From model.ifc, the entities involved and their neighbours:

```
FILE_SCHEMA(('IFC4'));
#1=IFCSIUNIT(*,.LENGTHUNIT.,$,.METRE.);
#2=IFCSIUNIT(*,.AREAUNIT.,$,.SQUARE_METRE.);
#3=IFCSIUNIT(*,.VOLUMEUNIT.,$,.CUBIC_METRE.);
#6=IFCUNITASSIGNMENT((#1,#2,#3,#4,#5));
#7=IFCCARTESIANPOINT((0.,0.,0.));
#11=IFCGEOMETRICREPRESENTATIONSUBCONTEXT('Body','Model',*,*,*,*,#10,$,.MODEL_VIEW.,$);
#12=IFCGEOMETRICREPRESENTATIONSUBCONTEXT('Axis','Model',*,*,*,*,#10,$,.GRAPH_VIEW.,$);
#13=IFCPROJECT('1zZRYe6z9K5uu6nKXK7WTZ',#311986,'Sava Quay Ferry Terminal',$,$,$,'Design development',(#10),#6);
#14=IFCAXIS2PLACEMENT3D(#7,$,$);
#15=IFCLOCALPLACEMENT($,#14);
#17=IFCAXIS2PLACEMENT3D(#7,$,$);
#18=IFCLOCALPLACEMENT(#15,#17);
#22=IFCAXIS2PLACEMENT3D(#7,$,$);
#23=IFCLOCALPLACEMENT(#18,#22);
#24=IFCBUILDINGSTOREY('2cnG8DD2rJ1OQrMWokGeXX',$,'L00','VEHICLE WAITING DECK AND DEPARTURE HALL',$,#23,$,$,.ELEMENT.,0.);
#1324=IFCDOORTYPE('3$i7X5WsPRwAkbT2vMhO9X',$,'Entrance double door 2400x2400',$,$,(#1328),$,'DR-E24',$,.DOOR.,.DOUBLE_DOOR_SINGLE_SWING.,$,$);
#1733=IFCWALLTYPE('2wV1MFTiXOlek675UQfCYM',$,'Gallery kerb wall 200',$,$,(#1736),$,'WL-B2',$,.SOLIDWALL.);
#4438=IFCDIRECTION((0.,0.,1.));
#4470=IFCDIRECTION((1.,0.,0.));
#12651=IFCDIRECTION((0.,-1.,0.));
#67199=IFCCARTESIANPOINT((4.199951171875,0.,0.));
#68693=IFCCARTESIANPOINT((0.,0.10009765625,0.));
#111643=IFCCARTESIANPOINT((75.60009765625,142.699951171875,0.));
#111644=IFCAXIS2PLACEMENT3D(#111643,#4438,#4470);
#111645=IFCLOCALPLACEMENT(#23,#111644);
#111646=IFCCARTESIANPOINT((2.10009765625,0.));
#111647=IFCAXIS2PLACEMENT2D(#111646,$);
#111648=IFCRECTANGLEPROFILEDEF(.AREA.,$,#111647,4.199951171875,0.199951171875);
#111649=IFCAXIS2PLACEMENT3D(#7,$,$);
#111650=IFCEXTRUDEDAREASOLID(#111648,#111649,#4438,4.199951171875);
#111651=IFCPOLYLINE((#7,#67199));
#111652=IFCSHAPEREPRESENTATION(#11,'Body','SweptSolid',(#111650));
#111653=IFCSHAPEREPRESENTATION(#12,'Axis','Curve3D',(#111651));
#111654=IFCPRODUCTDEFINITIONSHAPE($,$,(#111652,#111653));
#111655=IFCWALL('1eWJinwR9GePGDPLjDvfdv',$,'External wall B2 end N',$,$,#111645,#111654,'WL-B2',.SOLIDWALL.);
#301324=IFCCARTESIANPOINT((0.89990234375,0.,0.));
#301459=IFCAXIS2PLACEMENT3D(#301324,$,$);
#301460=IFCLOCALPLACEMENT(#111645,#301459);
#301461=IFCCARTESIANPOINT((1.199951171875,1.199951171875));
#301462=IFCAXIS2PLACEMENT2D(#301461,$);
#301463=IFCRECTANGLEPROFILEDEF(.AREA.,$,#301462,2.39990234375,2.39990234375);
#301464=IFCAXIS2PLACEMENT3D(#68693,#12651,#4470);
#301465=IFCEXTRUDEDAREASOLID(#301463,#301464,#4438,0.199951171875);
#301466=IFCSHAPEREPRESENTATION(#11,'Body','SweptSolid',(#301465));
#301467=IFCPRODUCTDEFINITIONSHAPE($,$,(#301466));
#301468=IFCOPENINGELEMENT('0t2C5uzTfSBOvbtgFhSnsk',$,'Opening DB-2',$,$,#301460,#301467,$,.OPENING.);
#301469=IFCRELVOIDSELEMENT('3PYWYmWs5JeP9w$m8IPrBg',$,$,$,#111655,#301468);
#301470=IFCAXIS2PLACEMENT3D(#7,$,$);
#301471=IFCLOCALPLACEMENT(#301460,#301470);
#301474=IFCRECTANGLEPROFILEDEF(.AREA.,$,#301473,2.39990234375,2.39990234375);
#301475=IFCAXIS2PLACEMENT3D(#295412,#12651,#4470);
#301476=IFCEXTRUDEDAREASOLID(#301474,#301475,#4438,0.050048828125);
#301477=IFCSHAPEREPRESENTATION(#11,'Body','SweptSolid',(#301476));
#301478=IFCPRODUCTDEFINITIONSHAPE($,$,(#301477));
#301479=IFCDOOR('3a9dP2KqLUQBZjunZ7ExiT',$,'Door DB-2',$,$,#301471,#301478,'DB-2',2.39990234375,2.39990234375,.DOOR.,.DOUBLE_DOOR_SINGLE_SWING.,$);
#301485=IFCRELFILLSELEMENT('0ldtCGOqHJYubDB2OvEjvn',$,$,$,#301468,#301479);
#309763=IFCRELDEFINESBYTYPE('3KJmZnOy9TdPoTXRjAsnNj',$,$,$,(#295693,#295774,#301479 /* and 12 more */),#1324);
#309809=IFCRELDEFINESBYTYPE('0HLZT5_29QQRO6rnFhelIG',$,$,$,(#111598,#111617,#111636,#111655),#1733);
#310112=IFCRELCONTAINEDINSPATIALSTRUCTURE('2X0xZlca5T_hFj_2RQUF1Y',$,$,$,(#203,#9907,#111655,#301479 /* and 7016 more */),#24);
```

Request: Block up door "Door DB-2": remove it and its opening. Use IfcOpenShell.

```python
import ifcopenshell
import ifcopenshell.api.feature
import ifcopenshell.api.root
import ifcopenshell.geom
import ifcopenshell.util.shape

model = ifcopenshell.open("model.ifc")
settings = ifcopenshell.geom.settings()


def volume(element):
    """Net volume in cubic metres, openings subtracted."""
    shape = ifcopenshell.geom.create_shape(settings, element)
    return ifcopenshell.util.shape.get_volume(shape.geometry)


door = model.by_guid("3a9dP2KqLUQBZjunZ7ExiT")
opening = door.FillsVoids[0].RelatingOpeningElement
wall = opening.VoidsElements[0].RelatingBuildingElement
before = volume(wall)

ifcopenshell.api.root.remove_product(model, product=door)
ifcopenshell.api.feature.remove_feature(model, feature=opening)

after = volume(wall)

print(f"wall volume {before:.3f} -> {after:.3f} m3")

model.write("model_updated.ifc")
```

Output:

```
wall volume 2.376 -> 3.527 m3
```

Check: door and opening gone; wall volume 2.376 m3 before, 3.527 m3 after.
